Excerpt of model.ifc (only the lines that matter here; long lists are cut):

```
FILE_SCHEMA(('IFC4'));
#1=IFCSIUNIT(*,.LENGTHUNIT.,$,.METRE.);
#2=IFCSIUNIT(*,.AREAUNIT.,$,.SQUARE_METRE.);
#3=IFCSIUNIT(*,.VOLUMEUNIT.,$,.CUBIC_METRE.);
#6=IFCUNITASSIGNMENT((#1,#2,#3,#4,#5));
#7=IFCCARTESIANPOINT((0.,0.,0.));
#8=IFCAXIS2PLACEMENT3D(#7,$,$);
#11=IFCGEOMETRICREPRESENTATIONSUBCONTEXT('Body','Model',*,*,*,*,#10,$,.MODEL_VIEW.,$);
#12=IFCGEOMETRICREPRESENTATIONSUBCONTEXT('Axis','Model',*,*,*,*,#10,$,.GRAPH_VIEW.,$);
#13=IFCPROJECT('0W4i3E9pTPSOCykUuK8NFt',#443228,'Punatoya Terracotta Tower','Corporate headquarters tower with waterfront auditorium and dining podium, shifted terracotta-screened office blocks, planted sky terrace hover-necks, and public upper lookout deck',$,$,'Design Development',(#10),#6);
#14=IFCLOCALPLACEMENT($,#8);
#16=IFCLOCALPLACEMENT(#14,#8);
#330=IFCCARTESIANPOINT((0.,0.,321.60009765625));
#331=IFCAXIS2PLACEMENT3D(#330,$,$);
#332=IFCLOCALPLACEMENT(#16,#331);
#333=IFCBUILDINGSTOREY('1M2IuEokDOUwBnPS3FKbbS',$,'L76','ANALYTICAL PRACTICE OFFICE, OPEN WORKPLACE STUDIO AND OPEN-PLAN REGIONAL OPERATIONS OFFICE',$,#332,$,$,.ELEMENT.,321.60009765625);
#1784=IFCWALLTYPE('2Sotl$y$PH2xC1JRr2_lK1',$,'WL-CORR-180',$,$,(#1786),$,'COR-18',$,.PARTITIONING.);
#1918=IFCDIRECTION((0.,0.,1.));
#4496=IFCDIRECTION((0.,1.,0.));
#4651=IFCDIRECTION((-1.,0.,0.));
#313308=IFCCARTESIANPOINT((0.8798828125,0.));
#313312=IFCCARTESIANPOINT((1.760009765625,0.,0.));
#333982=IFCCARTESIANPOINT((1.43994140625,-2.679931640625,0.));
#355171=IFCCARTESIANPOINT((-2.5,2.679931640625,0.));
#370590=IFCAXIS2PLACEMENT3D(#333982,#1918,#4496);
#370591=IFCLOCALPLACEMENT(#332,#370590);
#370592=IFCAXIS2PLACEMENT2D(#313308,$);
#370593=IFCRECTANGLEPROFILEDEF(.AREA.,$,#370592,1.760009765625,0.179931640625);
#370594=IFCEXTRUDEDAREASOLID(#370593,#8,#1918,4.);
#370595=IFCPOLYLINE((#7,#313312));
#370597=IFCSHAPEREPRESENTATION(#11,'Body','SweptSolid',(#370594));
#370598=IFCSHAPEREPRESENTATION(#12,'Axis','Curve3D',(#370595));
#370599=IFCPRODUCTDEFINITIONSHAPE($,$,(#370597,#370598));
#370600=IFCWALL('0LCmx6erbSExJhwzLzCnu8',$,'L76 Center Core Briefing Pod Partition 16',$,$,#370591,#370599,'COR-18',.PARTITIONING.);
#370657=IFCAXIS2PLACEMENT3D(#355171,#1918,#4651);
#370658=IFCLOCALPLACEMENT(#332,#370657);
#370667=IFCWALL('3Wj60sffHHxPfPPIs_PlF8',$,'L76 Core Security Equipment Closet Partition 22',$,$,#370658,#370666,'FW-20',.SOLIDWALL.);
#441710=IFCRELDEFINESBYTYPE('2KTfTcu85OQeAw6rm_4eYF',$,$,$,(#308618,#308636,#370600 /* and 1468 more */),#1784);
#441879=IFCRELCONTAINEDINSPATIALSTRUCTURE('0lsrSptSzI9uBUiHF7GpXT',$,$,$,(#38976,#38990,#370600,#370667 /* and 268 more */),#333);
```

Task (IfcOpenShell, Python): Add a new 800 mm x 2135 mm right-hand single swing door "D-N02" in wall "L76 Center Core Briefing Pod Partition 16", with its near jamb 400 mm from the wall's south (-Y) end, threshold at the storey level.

```python
import numpy as np
import ifcopenshell
import ifcopenshell.api.feature
import ifcopenshell.api.geometry
import ifcopenshell.api.root
import ifcopenshell.api.spatial
import ifcopenshell.geom
import ifcopenshell.util.element
import ifcopenshell.util.placement
import ifcopenshell.util.representation
import ifcopenshell.util.shape
import ifcopenshell.util.unit

model = ifcopenshell.open("model.ifc")
unit_scale = ifcopenshell.util.unit.calculate_unit_scale(model)
settings = ifcopenshell.geom.settings()


def volume(element):
    """Net volume in cubic metres, openings subtracted."""
    shape = ifcopenshell.geom.create_shape(settings, element)
    return ifcopenshell.util.shape.get_volume(shape.geometry)


wall = model.by_guid("0LCmx6erbSExJhwzLzCnu8")
storey = ifcopenshell.util.element.get_container(wall, ifc_class="IfcBuildingStorey")
context = ifcopenshell.util.representation.get_context(model, "Model", "Body", "MODEL_VIEW")
before = volume(wall)

width, height, from_end, sill = 0.8, 2.135, 0.4, 0.0  # metres

# The wall runs along its own X axis, and the end named is its -X end.
wall_shape = ifcopenshell.geom.create_shape(settings, wall)
x, y, z = ifcopenshell.util.shape.get_vertices(wall_shape.geometry).T
start = x.min() + from_end
face, thickness = float(y.min()), float(y.max() - y.min())
wall_matrix = ifcopenshell.util.placement.get_local_placement(wall.ObjectPlacement)
level = ifcopenshell.util.placement.get_local_placement(storey.ObjectPlacement)[2, 3]


def in_wall(x, y):
    """Placement at x, y metres in the wall's axes, at sill height."""
    matrix = wall_matrix.copy()
    matrix[:, 3] = wall_matrix @ np.array([x / unit_scale, y / unit_scale, 0.0, 1.0])
    matrix[2, 3] = level + sill / unit_scale
    return matrix


# Opening: a box that overshoots both wall faces by 50 mm.
opening = ifcopenshell.api.root.create_entity(model, ifc_class="IfcOpeningElement", predefined_type="OPENING")
box = ifcopenshell.api.geometry.add_wall_representation(
    model, context=context, length=width, height=height, thickness=thickness + 0.1
)
ifcopenshell.api.geometry.assign_representation(model, product=opening, representation=box)
ifcopenshell.api.geometry.edit_object_placement(model, product=opening, matrix=in_wall(start, face - 0.05), is_si=False)
ifcopenshell.api.feature.add_feature(model, feature=opening, element=wall)

door = ifcopenshell.api.root.create_entity(model, ifc_class="IfcDoor", name="D-N02", predefined_type="DOOR")
door.OverallWidth, door.OverallHeight = width / unit_scale, height / unit_scale
door.OperationType = "SINGLE_SWING_RIGHT"
body = ifcopenshell.api.geometry.add_door_representation(
    model,
    context=context,
    overall_width=door.OverallWidth,
    overall_height=door.OverallHeight,
    operation_type="SINGLE_SWING_RIGHT",
    lining_properties={"LiningDepth": thickness / unit_scale, "ThresholdDepth": thickness / unit_scale},
)
ifcopenshell.api.geometry.assign_representation(model, product=door, representation=body)
ifcopenshell.api.spatial.assign_container(model, products=[door], relating_structure=storey)
ifcopenshell.api.feature.add_filling(model, opening=opening, element=door)

# The lining spans the wall, so the door starts at the wall face.
ifcopenshell.api.geometry.edit_object_placement(model, product=door, matrix=in_wall(start, face), is_si=False)

after = volume(wall)

print(f"wall volume {before:.3f} -> {after:.3f} m3")

model.write("model_updated.ifc")
```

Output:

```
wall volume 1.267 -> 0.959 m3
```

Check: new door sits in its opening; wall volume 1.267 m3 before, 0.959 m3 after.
